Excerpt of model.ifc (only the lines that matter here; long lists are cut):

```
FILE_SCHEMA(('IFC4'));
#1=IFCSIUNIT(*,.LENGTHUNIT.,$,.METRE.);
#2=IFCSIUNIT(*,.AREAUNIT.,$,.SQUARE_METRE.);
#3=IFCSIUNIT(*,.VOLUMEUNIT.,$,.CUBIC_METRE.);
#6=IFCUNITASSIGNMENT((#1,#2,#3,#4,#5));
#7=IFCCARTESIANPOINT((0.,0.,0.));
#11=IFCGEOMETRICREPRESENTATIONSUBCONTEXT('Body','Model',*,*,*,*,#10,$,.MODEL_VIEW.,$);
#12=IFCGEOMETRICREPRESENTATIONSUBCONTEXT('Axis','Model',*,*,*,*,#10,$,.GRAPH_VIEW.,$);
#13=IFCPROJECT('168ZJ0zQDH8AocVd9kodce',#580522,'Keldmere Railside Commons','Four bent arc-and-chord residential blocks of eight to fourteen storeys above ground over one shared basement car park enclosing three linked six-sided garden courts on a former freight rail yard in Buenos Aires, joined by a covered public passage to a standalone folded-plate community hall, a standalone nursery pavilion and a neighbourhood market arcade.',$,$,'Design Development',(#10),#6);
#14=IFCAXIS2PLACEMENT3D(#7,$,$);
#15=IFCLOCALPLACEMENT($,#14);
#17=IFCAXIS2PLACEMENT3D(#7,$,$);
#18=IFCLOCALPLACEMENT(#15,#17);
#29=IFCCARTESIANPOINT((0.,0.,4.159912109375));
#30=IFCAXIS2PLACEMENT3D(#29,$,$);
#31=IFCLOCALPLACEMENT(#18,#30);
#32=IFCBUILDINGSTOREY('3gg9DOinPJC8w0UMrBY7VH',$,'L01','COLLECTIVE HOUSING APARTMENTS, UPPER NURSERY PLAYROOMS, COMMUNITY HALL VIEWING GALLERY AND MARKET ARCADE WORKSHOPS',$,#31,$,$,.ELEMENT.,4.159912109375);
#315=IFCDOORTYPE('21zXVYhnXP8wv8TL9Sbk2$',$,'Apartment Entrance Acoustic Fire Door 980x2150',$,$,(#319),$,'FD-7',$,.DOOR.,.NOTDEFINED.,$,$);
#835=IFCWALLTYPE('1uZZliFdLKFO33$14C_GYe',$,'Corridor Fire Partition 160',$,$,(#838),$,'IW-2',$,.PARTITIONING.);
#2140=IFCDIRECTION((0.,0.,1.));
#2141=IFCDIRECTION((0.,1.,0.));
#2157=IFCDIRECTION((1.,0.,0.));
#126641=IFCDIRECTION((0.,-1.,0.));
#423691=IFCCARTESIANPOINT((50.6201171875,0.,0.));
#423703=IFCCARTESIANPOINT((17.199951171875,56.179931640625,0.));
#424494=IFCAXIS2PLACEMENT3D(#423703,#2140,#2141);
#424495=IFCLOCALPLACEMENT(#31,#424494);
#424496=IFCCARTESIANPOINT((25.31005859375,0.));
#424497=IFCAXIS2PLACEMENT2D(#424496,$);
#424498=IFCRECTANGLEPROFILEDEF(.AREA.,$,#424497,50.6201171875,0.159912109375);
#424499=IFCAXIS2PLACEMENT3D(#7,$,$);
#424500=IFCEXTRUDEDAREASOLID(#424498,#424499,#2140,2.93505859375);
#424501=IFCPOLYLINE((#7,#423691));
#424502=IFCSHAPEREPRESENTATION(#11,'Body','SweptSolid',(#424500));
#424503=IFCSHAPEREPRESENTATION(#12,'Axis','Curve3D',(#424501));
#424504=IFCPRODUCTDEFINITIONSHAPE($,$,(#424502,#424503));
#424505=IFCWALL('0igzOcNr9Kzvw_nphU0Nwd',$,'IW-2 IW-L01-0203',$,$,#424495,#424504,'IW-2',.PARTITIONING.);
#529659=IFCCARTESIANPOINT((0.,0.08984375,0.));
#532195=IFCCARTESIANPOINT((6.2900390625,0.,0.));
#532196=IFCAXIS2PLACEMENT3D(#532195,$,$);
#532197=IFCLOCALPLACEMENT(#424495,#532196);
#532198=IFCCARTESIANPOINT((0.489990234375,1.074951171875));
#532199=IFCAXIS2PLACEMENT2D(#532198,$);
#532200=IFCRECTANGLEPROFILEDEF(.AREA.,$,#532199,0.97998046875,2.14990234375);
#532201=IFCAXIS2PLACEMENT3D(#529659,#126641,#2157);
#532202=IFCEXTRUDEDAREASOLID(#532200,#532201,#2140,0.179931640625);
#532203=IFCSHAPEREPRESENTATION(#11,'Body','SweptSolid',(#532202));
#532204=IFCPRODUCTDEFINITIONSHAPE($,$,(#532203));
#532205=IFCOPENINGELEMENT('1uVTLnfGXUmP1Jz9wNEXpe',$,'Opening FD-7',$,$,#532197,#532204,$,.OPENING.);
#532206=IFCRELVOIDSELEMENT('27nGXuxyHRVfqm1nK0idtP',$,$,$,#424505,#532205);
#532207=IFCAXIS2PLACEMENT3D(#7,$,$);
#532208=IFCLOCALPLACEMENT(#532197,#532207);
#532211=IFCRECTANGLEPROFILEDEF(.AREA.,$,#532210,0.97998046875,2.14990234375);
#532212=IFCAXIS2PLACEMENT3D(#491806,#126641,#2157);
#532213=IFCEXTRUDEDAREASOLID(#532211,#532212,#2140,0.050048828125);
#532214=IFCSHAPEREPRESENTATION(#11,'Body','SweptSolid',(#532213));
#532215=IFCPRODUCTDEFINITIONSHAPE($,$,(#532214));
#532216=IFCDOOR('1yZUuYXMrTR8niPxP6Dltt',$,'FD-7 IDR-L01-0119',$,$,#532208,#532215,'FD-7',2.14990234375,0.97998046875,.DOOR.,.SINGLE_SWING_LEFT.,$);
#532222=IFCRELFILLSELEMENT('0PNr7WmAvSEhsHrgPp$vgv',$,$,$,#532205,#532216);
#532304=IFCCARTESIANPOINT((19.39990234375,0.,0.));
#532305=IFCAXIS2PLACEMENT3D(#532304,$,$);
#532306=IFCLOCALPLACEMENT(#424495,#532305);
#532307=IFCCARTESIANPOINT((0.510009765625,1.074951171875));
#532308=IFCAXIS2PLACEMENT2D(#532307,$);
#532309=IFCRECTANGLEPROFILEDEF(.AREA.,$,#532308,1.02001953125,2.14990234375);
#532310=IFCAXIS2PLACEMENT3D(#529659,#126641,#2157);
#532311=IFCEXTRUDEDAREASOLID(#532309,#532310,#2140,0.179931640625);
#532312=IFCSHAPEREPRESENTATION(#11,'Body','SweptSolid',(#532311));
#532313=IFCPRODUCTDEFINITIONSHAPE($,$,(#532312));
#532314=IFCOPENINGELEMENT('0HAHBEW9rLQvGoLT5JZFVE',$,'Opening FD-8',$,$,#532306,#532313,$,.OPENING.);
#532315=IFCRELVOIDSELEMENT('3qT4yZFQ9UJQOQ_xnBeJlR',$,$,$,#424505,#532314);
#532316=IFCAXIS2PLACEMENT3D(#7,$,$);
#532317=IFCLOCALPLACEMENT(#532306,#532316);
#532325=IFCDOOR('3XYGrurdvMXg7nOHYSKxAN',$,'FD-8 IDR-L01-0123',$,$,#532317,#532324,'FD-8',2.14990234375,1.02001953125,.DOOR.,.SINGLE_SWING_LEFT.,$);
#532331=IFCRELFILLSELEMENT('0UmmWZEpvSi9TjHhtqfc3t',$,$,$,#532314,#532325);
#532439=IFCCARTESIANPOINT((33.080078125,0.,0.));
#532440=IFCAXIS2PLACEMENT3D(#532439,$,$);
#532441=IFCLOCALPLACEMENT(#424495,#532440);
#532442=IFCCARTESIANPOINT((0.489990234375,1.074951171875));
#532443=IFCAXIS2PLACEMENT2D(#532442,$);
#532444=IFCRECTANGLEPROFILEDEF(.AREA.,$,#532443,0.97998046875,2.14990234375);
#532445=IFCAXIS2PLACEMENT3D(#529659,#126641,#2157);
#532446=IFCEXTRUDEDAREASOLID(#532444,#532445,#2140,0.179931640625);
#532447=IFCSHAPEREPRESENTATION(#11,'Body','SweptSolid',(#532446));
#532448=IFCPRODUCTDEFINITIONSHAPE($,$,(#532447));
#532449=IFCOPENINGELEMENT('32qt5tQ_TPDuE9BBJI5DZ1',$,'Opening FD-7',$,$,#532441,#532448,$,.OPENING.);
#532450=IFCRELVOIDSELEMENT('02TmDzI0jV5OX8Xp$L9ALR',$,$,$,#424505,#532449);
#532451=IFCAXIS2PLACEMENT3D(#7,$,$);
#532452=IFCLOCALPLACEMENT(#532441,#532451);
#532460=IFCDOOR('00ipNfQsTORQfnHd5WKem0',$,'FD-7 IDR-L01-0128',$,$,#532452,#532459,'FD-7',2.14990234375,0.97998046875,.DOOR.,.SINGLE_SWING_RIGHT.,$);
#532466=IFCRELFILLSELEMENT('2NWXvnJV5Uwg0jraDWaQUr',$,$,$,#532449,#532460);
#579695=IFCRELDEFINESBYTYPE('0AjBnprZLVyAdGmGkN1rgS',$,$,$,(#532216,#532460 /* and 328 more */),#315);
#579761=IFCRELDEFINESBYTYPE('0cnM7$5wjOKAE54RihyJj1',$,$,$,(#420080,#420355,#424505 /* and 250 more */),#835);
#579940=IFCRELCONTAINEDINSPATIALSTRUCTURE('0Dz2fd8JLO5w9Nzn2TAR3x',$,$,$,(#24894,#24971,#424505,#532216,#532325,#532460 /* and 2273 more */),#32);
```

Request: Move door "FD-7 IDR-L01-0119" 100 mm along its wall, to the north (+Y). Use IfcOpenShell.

```python
import ifcopenshell
import ifcopenshell.api.geometry
import ifcopenshell.util.placement

model = ifcopenshell.open("model.ifc")

door = model.by_guid("1yZUuYXMrTR8niPxP6Dltt")
opening = door.FillsVoids[0].RelatingOpeningElement
wall = opening.VoidsElements[0].RelatingBuildingElement

wall_matrix = ifcopenshell.util.placement.get_local_placement(wall.ObjectPlacement)
shift = wall_matrix[:3, 0] * 0.1
before = ifcopenshell.util.placement.get_local_placement(door.ObjectPlacement)[:3, 3].copy()

# The door is placed relative to its opening, so it follows when the opening moves.
matrix = ifcopenshell.util.placement.get_local_placement(opening.ObjectPlacement)
matrix[:3, 3] += shift
ifcopenshell.api.geometry.edit_object_placement(
    model, product=opening, matrix=matrix, is_si=False, should_transform_children=True
)

after = ifcopenshell.util.placement.get_local_placement(door.ObjectPlacement)[:3, 3]
print("door moved by", (after - before).round(3) + 0.0)

model.write("model-out.ifc")
```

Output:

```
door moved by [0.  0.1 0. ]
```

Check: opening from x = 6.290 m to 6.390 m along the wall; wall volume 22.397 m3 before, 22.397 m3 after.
